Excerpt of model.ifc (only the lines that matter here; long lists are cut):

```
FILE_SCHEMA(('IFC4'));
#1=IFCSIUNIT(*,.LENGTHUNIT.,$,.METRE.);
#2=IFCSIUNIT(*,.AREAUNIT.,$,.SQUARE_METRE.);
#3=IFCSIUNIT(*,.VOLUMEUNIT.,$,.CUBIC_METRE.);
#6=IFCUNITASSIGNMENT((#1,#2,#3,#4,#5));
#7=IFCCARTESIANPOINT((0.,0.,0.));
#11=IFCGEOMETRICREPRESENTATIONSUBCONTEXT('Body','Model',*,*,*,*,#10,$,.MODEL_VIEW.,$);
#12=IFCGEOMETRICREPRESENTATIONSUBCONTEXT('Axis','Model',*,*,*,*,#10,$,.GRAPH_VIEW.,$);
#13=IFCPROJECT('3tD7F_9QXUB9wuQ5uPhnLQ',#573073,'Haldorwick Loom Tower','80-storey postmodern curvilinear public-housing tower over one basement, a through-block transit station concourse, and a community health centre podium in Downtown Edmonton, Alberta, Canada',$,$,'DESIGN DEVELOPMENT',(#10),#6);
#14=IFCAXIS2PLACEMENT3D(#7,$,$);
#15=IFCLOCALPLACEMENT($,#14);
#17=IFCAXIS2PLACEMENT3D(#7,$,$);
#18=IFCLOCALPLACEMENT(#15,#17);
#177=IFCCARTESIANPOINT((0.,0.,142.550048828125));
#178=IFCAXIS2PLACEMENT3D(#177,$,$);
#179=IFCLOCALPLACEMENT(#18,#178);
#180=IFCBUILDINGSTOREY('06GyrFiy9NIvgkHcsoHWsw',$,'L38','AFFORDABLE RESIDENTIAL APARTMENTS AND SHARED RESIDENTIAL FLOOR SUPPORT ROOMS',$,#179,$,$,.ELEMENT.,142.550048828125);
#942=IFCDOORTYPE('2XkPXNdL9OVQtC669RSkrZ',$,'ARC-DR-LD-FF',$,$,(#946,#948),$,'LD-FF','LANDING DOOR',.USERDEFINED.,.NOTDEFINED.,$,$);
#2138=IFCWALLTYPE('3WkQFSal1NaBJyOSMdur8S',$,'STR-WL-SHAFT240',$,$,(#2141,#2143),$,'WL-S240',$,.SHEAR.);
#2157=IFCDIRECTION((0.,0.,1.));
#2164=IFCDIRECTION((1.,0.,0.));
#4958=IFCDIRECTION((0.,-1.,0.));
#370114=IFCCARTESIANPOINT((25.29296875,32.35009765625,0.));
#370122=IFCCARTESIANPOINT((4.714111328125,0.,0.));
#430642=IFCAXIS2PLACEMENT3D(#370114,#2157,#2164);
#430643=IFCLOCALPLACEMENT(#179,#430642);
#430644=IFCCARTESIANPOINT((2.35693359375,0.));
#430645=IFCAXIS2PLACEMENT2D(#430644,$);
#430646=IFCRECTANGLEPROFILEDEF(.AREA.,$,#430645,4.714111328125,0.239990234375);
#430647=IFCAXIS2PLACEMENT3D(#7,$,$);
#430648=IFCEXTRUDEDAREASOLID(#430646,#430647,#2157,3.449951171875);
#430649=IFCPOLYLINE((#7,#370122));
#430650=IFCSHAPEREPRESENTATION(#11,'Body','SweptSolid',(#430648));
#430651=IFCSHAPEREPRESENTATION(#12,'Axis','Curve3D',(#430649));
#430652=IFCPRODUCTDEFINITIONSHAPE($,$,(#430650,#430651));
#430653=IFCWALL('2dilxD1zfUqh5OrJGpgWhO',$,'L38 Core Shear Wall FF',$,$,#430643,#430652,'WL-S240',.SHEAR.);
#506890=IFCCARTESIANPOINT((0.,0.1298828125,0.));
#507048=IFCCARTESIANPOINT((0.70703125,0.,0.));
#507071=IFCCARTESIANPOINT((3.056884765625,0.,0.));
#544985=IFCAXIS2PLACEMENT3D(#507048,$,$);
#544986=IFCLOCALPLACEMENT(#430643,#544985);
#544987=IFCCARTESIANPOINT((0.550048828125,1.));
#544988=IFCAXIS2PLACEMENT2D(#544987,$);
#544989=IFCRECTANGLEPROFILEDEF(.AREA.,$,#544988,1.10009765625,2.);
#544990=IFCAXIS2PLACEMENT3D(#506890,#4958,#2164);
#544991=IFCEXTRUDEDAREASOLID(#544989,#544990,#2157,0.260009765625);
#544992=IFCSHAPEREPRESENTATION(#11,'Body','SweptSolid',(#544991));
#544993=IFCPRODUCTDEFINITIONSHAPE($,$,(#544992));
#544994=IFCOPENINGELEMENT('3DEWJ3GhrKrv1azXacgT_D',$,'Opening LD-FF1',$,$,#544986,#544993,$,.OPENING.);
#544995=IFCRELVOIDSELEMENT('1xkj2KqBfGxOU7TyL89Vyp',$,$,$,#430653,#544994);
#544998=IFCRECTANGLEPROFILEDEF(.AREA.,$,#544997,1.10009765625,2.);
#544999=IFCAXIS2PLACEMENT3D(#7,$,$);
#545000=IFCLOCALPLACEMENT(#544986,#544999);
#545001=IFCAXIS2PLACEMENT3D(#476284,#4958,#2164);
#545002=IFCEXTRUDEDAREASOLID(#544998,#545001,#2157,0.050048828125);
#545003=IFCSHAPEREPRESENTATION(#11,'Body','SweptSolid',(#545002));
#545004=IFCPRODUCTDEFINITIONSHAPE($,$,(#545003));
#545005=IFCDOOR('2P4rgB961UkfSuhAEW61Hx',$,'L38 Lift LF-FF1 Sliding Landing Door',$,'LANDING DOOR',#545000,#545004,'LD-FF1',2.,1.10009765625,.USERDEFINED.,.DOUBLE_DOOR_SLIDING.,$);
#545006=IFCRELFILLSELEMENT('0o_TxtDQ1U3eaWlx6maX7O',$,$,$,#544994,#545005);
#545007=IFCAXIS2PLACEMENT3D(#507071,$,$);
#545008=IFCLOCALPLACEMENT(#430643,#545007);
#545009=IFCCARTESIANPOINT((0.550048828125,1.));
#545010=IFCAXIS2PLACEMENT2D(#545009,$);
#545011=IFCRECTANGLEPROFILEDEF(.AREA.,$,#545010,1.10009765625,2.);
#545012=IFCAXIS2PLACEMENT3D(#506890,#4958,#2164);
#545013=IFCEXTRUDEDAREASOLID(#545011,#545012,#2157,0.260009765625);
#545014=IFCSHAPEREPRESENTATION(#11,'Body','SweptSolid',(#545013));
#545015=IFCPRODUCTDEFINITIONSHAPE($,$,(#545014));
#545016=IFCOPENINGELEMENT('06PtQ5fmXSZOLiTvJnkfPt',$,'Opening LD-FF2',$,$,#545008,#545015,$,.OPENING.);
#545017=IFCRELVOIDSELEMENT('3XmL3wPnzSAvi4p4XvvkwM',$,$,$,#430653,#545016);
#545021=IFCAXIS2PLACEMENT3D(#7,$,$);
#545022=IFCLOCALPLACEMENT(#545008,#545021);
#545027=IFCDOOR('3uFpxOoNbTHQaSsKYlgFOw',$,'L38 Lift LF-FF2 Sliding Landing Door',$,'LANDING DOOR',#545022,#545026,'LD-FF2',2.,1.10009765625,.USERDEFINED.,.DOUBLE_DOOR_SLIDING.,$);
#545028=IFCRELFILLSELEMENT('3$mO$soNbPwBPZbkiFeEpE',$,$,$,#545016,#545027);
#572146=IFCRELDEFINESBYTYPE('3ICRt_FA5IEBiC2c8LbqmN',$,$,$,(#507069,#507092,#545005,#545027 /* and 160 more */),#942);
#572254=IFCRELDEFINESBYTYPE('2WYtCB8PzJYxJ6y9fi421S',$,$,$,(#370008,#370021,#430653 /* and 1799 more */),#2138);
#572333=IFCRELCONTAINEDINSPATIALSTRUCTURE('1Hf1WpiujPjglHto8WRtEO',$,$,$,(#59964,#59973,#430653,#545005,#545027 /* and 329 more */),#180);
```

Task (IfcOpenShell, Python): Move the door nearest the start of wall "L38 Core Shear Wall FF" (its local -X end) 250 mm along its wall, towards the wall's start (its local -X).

```python
import ifcopenshell
import ifcopenshell.api.geometry
import ifcopenshell.util.placement
import ifcopenshell.util.unit

model = ifcopenshell.open("model.ifc")
unit_scale = ifcopenshell.util.unit.calculate_unit_scale(model)

door = model.by_guid("2P4rgB961UkfSuhAEW61Hx")
opening = door.FillsVoids[0].RelatingOpeningElement
wall = opening.VoidsElements[0].RelatingBuildingElement

wall_matrix = ifcopenshell.util.placement.get_local_placement(wall.ObjectPlacement)
shift = wall_matrix[:3, 0] * -0.25 / unit_scale
before = ifcopenshell.util.placement.get_local_placement(door.ObjectPlacement)[:3, 3].copy()

# The door is placed relative to its opening, so it follows when the opening moves.
matrix = ifcopenshell.util.placement.get_local_placement(opening.ObjectPlacement)
matrix[:3, 3] += shift
ifcopenshell.api.geometry.edit_object_placement(
    model, product=opening, matrix=matrix, is_si=False, should_transform_children=True
)

after = ifcopenshell.util.placement.get_local_placement(door.ObjectPlacement)[:3, 3]
print("door moved by", (after - before).round(3) + 0.0)

model.write("model_rev.ifc")
```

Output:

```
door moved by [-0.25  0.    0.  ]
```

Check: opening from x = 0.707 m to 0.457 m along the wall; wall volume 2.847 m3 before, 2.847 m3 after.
